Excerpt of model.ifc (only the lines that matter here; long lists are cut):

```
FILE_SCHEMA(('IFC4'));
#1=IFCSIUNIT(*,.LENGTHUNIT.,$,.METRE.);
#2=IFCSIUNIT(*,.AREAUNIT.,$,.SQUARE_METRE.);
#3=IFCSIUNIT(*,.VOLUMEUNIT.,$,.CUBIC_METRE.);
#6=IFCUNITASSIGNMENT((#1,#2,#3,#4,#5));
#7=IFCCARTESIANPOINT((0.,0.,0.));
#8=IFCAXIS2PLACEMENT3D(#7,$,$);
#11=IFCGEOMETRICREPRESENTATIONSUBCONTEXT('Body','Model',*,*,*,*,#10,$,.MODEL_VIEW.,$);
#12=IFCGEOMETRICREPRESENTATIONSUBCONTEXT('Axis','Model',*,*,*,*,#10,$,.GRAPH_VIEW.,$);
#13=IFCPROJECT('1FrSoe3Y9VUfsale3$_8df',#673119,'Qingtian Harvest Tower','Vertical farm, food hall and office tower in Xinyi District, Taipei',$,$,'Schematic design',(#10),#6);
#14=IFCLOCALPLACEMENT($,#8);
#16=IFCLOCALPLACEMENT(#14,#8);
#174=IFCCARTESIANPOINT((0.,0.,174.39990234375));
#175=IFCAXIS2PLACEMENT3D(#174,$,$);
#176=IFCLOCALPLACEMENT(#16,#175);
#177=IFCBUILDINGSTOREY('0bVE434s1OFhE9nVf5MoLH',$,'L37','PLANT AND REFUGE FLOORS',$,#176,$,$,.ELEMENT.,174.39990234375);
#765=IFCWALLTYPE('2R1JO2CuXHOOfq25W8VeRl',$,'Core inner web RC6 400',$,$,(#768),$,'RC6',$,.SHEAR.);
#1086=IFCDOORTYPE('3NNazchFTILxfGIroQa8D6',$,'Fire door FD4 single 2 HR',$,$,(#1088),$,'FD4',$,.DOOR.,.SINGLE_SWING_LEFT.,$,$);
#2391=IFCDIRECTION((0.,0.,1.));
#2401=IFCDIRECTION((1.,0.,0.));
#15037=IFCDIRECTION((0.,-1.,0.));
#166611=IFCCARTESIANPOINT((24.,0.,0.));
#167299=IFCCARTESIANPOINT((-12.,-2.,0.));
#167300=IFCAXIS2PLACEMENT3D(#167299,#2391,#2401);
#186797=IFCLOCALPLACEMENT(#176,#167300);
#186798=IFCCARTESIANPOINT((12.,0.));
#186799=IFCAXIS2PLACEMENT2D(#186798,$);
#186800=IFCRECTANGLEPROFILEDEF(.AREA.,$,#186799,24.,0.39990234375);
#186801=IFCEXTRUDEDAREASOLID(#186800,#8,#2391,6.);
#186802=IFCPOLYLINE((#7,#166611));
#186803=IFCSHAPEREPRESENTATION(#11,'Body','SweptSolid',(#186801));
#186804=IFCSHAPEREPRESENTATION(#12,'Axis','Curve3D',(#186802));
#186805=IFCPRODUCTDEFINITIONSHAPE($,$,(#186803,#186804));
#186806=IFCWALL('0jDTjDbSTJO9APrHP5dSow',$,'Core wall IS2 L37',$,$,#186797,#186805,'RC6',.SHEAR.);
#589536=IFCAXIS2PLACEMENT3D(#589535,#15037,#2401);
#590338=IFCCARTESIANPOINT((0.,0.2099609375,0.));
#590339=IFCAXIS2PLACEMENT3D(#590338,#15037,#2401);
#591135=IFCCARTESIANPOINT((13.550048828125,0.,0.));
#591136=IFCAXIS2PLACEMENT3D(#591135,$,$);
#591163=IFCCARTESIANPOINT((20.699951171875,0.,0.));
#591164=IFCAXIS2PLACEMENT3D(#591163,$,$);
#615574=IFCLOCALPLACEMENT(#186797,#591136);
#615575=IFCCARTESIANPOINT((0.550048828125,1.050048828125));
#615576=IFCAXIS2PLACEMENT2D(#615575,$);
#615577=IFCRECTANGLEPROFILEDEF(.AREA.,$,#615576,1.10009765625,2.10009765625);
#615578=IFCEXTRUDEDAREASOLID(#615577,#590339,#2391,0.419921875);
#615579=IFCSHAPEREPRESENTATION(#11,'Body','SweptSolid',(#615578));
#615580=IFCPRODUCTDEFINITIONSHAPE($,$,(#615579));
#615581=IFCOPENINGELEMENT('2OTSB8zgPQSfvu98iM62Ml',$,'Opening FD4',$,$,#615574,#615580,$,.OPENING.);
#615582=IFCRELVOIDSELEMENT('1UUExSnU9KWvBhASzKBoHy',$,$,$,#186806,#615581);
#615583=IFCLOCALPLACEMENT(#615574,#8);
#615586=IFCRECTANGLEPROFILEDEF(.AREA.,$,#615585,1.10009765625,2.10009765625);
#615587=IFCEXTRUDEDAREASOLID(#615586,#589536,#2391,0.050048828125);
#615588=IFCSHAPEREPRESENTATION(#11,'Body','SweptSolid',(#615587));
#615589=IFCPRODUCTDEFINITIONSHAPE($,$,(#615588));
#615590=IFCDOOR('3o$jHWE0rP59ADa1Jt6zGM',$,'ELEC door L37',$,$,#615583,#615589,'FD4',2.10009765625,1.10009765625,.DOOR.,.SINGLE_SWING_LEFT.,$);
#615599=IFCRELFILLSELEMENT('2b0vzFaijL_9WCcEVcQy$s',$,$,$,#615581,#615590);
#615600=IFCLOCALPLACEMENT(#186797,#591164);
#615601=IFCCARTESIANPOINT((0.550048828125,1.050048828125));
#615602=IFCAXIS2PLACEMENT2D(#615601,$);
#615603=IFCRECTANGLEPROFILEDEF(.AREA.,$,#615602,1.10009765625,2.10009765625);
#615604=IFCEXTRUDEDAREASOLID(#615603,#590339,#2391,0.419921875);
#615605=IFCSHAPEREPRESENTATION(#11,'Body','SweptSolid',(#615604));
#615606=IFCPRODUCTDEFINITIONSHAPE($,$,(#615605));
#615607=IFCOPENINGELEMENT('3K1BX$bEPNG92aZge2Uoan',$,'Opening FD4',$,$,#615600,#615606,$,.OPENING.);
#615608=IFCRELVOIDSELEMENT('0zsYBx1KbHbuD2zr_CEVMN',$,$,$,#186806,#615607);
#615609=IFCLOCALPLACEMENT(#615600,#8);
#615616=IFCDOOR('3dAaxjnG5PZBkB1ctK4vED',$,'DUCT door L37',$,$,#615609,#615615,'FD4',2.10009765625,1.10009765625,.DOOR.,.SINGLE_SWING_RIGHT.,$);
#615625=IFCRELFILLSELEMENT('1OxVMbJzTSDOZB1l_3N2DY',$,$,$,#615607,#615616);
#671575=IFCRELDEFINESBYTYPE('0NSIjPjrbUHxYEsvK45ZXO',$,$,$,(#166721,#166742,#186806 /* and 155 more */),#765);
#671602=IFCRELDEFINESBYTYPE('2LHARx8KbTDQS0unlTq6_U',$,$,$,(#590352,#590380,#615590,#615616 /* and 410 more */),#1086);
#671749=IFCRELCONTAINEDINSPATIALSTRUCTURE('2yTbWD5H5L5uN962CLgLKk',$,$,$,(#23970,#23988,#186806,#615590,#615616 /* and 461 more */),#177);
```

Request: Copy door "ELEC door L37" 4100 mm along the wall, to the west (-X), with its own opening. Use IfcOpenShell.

```python
import ifcopenshell
import ifcopenshell.api.feature
import ifcopenshell.api.geometry
import ifcopenshell.api.root
import ifcopenshell.geom
import ifcopenshell.util.element
import ifcopenshell.util.placement
import ifcopenshell.util.shape
import ifcopenshell.util.unit

model = ifcopenshell.open("model.ifc")
unit_scale = ifcopenshell.util.unit.calculate_unit_scale(model)
settings = ifcopenshell.geom.settings()


def volume(element):
    """Net volume in cubic metres, openings subtracted."""
    shape = ifcopenshell.geom.create_shape(settings, element)
    return ifcopenshell.util.shape.get_volume(shape.geometry)


door = model.by_id(615590)
opening = door.FillsVoids[0].RelatingOpeningElement
wall = opening.VoidsElements[0].RelatingBuildingElement
before = volume(wall)
shift = ifcopenshell.util.placement.get_local_placement(wall.ObjectPlacement)[:3, 0] * -4.1 / unit_scale

# copy_class copies the void relationship, type, container and properties, but no geometry.
new_opening = ifcopenshell.api.root.copy_class(model, product=opening)
new_opening.Representation = ifcopenshell.util.element.copy_deep(
    model, opening.Representation, exclude=["IfcGeometricRepresentationContext", "IfcRepresentationMap"]
)
new_door = ifcopenshell.api.root.copy_class(model, product=door)
new_door.Representation = ifcopenshell.util.element.copy_deep(
    model, door.Representation, exclude=["IfcGeometricRepresentationContext", "IfcRepresentationMap"]
)
new_door.Tag = None
ifcopenshell.api.feature.add_filling(model, opening=new_opening, element=new_door)

for old, new in ((opening, new_opening), (door, new_door)):
    matrix = ifcopenshell.util.placement.get_local_placement(old.ObjectPlacement)
    matrix[:3, 3] += shift
    ifcopenshell.api.geometry.edit_object_placement(model, product=new, matrix=matrix, is_si=False)

after = volume(wall)

print(f"wall volume {before:.3f} -> {after:.3f} m3")

model.write("model_updated.ifc")
```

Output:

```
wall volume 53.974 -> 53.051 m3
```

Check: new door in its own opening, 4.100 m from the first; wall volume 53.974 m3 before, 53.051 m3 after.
